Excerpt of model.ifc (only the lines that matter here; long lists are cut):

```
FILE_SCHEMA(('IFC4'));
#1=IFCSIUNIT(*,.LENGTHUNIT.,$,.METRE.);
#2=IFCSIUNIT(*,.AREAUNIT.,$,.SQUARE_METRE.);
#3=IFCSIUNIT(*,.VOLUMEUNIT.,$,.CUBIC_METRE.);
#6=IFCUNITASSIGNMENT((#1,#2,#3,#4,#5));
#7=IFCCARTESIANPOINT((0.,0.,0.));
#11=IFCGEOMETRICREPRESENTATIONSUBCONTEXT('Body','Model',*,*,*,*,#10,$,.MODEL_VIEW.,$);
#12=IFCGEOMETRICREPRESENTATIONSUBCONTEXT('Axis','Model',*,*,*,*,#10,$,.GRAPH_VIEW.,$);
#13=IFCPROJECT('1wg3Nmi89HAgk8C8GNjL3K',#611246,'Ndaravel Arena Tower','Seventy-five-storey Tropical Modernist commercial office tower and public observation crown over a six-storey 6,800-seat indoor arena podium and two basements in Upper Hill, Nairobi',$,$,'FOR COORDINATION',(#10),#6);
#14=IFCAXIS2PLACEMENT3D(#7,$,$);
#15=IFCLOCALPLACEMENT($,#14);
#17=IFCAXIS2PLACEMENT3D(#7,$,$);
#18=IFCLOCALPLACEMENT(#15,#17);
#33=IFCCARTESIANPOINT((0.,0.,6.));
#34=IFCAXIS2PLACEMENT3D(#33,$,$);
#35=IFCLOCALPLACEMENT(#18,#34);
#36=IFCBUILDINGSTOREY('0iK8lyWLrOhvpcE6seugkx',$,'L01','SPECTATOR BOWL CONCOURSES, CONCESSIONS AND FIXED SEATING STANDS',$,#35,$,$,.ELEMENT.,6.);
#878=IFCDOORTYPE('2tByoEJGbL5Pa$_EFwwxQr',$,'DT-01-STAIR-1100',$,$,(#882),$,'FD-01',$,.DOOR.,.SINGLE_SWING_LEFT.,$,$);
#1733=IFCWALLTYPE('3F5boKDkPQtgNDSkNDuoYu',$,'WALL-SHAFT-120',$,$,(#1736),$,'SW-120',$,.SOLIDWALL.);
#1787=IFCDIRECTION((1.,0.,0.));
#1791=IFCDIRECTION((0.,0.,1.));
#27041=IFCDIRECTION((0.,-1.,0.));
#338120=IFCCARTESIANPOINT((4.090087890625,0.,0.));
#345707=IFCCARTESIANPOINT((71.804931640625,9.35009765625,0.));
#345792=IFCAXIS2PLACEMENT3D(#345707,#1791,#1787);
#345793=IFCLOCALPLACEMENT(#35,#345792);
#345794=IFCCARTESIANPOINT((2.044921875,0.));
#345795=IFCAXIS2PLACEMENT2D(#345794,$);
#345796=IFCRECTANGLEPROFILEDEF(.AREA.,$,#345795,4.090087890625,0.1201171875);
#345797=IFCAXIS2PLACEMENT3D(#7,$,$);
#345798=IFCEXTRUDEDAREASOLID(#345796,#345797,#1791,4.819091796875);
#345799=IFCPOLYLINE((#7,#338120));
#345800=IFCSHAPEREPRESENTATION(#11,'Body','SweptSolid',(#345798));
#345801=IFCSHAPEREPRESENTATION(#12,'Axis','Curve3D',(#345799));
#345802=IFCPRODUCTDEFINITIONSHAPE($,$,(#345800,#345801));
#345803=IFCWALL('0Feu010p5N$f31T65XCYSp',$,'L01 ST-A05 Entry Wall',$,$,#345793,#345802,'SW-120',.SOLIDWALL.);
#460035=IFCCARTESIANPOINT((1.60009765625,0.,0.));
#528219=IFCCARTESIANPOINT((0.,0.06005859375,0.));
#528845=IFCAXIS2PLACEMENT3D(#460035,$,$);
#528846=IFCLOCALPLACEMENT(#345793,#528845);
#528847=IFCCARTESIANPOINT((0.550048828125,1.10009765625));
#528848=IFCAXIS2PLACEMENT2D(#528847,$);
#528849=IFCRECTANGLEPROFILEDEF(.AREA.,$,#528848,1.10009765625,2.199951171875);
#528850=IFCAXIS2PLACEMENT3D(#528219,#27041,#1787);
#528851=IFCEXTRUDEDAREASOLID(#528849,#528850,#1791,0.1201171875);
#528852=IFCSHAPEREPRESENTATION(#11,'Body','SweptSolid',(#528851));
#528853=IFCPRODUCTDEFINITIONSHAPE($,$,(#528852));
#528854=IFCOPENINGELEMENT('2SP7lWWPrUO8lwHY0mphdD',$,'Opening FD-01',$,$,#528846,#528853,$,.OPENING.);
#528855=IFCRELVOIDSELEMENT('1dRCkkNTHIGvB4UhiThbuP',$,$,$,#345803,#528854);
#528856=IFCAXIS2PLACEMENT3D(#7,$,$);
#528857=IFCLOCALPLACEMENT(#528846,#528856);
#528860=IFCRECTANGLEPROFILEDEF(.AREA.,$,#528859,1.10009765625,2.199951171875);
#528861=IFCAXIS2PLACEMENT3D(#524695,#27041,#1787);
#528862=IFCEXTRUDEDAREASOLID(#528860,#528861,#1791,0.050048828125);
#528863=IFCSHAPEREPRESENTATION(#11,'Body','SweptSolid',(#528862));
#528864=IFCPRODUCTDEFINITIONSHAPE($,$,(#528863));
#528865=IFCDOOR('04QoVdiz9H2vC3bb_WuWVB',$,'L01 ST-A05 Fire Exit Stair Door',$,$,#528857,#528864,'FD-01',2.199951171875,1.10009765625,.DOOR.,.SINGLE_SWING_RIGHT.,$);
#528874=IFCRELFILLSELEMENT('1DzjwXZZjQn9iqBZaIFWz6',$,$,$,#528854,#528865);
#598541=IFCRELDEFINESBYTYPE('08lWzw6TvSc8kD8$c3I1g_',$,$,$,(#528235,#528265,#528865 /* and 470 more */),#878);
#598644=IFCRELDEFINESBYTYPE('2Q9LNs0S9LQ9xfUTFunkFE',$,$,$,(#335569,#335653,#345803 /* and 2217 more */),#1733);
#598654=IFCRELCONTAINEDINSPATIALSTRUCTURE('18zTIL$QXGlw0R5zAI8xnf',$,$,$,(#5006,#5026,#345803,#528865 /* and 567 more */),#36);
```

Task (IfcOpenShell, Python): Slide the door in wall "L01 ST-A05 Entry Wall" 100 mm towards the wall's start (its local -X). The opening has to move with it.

```python
import ifcopenshell
import ifcopenshell.api.geometry
import ifcopenshell.util.placement
import ifcopenshell.util.unit

model = ifcopenshell.open("model.ifc")
unit_scale = ifcopenshell.util.unit.calculate_unit_scale(model)

door = model.by_guid("04QoVdiz9H2vC3bb_WuWVB")
opening = door.FillsVoids[0].RelatingOpeningElement
wall = opening.VoidsElements[0].RelatingBuildingElement

wall_matrix = ifcopenshell.util.placement.get_local_placement(wall.ObjectPlacement)
shift = wall_matrix[:3, 0] * -0.1 / unit_scale
before = ifcopenshell.util.placement.get_local_placement(door.ObjectPlacement)[:3, 3].copy()

# The door is placed relative to its opening, so it follows when the opening moves.
matrix = ifcopenshell.util.placement.get_local_placement(opening.ObjectPlacement)
matrix[:3, 3] += shift
ifcopenshell.api.geometry.edit_object_placement(
    model, product=opening, matrix=matrix, is_si=False, should_transform_children=True
)

after = ifcopenshell.util.placement.get_local_placement(door.ObjectPlacement)[:3, 3]
print("door moved by", (after - before).round(3) + 0.0)

model.write("model_edited.ifc")
```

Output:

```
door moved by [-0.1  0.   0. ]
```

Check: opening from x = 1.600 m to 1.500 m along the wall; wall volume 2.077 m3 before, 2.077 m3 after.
